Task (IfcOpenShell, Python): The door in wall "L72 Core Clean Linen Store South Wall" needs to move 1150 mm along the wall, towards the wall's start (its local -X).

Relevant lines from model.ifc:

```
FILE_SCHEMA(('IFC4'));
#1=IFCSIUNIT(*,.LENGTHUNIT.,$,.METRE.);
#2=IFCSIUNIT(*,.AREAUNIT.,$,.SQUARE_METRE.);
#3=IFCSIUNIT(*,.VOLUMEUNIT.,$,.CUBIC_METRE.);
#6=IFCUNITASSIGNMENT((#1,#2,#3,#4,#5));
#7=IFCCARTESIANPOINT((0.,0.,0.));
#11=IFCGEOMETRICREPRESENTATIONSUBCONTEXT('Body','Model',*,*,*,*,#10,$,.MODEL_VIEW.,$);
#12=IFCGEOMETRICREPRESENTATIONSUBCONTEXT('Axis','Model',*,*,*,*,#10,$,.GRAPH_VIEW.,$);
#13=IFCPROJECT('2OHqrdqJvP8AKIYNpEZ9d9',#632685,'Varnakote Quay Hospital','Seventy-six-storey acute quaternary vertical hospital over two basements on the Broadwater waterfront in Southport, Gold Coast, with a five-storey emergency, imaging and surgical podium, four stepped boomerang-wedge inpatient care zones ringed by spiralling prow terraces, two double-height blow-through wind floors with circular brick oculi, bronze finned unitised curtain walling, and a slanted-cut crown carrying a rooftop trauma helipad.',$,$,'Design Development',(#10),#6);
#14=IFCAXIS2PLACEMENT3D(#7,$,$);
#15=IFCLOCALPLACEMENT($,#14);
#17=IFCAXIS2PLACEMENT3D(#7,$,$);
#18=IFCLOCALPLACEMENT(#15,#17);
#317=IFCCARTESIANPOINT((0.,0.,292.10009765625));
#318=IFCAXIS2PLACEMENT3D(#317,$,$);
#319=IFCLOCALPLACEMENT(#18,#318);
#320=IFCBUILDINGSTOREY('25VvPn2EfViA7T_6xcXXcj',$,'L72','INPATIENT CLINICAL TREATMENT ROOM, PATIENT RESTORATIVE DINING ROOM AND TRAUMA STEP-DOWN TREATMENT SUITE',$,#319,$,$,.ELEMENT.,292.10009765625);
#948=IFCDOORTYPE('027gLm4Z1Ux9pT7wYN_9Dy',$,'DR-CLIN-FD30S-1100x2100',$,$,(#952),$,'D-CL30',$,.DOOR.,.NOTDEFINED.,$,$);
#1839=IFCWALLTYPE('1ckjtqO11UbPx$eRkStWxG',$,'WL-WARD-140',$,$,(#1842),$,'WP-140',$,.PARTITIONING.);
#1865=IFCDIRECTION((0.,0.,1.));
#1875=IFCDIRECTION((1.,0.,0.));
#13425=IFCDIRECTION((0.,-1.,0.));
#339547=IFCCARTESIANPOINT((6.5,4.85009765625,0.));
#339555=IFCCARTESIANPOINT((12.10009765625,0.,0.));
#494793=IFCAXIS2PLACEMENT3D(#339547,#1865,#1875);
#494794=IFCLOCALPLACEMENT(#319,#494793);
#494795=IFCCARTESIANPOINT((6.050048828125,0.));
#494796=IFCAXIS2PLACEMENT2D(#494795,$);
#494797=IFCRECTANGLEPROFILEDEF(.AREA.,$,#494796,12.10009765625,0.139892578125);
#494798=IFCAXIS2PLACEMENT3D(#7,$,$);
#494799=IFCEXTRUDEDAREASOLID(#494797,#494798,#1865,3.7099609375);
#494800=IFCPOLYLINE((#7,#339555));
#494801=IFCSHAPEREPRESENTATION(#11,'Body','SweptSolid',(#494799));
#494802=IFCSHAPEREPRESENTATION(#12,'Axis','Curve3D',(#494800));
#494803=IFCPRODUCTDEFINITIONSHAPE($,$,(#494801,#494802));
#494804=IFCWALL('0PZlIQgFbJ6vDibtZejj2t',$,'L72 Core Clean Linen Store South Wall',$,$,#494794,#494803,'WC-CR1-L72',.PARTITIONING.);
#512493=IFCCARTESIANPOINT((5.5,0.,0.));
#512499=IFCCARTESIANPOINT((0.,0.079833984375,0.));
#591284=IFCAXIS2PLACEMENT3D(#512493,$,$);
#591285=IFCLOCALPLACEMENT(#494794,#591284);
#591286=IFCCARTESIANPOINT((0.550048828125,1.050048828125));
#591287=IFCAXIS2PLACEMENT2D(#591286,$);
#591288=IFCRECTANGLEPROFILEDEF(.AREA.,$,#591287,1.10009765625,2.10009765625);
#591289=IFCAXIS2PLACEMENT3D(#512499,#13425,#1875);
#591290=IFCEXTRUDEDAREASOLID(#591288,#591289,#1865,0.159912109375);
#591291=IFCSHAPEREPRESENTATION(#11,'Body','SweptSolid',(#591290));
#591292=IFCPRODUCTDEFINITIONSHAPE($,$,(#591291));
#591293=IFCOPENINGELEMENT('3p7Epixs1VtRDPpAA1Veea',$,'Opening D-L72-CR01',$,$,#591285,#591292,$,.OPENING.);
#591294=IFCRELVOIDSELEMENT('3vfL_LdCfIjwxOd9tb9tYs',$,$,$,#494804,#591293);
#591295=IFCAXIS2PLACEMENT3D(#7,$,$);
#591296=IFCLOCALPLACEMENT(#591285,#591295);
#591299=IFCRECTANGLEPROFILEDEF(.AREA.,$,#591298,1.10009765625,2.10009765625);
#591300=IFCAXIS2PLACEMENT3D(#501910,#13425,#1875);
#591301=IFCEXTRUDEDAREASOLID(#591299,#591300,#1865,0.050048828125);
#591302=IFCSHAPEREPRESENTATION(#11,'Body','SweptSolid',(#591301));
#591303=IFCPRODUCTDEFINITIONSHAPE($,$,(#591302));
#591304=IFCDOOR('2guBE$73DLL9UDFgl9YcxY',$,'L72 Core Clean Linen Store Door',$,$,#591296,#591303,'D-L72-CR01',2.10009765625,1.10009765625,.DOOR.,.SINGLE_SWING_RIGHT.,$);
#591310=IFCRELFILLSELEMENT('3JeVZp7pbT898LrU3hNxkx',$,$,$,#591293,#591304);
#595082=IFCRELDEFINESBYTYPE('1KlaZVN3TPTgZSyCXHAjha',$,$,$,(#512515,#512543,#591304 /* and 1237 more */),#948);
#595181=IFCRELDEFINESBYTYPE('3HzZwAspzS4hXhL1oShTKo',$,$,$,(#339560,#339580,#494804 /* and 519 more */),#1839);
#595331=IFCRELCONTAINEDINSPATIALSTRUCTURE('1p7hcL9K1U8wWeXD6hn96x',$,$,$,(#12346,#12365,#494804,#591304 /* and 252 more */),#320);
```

```python
import ifcopenshell
import ifcopenshell.api.geometry
import ifcopenshell.util.placement

model = ifcopenshell.open("model.ifc")

door = model.by_guid("2guBE$73DLL9UDFgl9YcxY")
opening = door.FillsVoids[0].RelatingOpeningElement
wall = opening.VoidsElements[0].RelatingBuildingElement

wall_matrix = ifcopenshell.util.placement.get_local_placement(wall.ObjectPlacement)
shift = wall_matrix[:3, 0] * -1.15
before = ifcopenshell.util.placement.get_local_placement(door.ObjectPlacement)[:3, 3].copy()

# The door is placed relative to its opening, so it follows when the opening moves.
matrix = ifcopenshell.util.placement.get_local_placement(opening.ObjectPlacement)
matrix[:3, 3] += shift
ifcopenshell.api.geometry.edit_object_placement(
    model, product=opening, matrix=matrix, is_si=False, should_transform_children=True
)

after = ifcopenshell.util.placement.get_local_placement(door.ObjectPlacement)[:3, 3]
print("door moved by", (after - before).round(3) + 0.0)

model.write("model_edited.ifc")
```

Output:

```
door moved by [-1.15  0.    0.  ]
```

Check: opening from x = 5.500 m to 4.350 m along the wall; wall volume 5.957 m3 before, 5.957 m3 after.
